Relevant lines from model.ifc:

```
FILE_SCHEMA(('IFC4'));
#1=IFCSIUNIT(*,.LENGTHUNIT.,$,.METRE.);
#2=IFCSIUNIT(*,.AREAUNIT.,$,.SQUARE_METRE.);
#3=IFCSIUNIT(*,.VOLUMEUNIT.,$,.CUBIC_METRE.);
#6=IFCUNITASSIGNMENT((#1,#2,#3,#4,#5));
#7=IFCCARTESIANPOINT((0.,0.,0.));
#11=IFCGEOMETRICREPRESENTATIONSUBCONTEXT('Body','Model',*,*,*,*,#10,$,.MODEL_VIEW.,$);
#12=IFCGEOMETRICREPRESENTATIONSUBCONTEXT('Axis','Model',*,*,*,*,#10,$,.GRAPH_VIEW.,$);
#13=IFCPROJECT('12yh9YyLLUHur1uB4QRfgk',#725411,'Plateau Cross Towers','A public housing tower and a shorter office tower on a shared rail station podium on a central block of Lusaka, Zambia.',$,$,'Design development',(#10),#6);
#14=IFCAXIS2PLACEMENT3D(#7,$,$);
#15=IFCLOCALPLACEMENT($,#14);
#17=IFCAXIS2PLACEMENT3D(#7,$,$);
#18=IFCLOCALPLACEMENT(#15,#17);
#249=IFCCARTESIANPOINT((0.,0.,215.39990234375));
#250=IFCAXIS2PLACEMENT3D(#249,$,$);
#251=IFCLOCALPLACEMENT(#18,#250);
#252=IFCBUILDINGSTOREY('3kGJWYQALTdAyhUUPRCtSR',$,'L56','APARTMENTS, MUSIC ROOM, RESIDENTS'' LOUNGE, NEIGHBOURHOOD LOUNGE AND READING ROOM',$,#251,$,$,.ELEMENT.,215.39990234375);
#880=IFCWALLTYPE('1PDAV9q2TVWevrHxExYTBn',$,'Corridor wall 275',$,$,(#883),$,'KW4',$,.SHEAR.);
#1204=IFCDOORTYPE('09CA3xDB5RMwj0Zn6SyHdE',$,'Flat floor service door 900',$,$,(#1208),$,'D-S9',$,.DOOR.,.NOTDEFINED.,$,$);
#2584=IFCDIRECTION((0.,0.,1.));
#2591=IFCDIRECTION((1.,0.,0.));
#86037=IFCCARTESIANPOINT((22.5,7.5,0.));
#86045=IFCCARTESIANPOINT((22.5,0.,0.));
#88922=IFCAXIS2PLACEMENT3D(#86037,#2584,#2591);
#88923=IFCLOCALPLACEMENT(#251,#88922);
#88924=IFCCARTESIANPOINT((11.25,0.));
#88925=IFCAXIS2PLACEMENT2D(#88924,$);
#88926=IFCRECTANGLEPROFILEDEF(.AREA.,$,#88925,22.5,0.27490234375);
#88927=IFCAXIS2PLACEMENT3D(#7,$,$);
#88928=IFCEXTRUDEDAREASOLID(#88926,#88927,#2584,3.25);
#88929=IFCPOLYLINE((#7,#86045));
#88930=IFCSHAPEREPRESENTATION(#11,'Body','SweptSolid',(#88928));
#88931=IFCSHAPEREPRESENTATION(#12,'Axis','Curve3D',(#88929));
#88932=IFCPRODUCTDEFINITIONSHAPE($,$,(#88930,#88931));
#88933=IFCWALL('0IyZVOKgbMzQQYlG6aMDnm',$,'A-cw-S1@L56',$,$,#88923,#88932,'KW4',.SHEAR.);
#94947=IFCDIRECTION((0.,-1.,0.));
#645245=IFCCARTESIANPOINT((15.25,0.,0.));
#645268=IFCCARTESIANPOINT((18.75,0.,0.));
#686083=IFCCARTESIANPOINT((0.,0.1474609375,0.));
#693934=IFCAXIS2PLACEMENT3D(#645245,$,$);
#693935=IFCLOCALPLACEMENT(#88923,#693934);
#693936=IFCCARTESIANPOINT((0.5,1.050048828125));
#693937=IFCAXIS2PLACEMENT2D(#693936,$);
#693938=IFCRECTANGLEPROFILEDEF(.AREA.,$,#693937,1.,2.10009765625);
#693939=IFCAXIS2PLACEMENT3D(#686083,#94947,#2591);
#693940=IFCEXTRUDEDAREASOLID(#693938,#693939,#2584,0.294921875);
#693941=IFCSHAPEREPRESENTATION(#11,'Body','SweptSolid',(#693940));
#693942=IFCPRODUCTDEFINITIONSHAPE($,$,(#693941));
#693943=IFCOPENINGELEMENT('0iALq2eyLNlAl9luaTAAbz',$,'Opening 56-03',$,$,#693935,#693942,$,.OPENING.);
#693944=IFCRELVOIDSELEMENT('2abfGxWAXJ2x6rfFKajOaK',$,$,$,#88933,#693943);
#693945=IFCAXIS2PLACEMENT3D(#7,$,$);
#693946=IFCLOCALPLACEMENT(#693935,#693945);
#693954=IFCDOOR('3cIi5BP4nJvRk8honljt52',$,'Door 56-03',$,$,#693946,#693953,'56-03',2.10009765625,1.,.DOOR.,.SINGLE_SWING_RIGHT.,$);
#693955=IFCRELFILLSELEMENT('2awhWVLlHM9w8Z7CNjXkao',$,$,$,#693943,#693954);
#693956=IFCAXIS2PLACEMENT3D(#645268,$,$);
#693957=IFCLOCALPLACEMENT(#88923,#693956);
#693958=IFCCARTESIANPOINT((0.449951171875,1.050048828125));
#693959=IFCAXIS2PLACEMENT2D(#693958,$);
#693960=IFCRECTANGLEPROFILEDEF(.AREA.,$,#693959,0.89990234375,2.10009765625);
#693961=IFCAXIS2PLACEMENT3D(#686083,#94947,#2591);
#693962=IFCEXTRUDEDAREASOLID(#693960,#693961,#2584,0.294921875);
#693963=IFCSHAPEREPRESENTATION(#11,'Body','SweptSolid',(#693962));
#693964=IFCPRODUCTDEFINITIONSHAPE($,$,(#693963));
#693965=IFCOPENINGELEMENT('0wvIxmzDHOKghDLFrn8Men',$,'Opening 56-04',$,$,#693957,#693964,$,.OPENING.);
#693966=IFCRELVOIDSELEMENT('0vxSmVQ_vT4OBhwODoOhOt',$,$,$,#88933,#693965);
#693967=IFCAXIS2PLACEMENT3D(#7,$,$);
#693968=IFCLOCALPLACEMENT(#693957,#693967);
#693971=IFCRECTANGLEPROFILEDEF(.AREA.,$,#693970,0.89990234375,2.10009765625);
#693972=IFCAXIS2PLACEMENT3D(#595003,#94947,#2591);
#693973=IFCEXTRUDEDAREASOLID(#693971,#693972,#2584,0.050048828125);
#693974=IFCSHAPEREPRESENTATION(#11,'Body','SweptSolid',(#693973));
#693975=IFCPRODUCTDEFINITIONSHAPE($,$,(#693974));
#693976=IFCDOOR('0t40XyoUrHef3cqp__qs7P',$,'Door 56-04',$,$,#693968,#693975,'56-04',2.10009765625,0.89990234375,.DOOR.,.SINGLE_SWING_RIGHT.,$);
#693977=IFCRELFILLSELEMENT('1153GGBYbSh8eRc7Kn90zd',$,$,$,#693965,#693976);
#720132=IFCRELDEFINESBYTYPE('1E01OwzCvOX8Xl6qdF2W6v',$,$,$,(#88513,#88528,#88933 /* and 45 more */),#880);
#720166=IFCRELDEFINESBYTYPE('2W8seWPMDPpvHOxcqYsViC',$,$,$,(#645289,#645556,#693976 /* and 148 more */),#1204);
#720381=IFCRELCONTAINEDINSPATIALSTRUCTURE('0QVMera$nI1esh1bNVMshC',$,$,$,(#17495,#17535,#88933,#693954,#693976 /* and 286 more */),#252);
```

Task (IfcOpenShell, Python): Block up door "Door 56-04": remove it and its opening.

```python
import ifcopenshell
import ifcopenshell.api.feature
import ifcopenshell.api.root
import ifcopenshell.geom
import ifcopenshell.util.shape

model = ifcopenshell.open("model.ifc")
settings = ifcopenshell.geom.settings()


def volume(element):
    """Net volume in cubic metres, openings subtracted."""
    shape = ifcopenshell.geom.create_shape(settings, element)
    return ifcopenshell.util.shape.get_volume(shape.geometry)


door = model.by_guid("0t40XyoUrHef3cqp__qs7P")
opening = door.FillsVoids[0].RelatingOpeningElement
wall = opening.VoidsElements[0].RelatingBuildingElement
before = volume(wall)

ifcopenshell.api.root.remove_product(model, product=door)
ifcopenshell.api.feature.remove_feature(model, feature=opening)

after = volume(wall)

print(f"wall volume {before:.3f} -> {after:.3f} m3")

model.write("model_rev.ifc")
```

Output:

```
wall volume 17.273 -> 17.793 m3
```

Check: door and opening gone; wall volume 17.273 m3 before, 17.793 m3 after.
